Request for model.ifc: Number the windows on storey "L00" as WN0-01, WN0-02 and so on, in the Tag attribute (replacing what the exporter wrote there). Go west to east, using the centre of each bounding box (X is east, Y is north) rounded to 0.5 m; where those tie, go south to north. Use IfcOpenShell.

First a look at what the model holds.

```python
import ifcopenshell
import ifcopenshell.util.element
import ifcopenshell.util.placement

model = ifcopenshell.open("model.ifc")
print(model.schema)
storey = next(s for s in model.by_type("IfcBuildingStorey") if s.Name == "L00")
windows = [e for e in ifcopenshell.util.element.get_decomposition(storey) if e.is_a("IfcWindow")]
for e in sorted(windows, key=lambda e: e.id()):
    origin = ifcopenshell.util.placement.get_local_placement(e.ObjectPlacement)[:3, 3]
    print(e.id(), e.Tag, e.Name, origin.round(2) + 0.0, sep=" | ")
```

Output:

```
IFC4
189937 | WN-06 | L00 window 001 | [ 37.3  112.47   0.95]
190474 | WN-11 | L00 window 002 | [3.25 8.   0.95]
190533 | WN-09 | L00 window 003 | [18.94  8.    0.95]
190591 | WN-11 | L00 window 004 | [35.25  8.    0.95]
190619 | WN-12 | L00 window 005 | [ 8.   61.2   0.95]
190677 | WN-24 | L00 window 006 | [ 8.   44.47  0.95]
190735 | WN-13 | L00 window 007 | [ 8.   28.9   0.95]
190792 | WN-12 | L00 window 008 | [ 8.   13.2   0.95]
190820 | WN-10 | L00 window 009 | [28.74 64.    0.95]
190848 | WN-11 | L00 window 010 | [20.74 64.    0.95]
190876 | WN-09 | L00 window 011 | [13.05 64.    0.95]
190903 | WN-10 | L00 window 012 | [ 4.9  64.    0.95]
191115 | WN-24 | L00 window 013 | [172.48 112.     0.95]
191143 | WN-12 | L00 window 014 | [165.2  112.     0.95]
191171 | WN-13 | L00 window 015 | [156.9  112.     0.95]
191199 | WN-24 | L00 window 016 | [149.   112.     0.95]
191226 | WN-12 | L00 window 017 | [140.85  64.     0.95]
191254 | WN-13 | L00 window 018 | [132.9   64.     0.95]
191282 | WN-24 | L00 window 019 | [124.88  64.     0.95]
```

```python
import ifcopenshell
import ifcopenshell.geom
import ifcopenshell.util.element
import ifcopenshell.util.shape

model = ifcopenshell.open("model.ifc")
settings = ifcopenshell.geom.settings()
settings.set("use-world-coords", True)


def centre(element):
    shape = ifcopenshell.geom.create_shape(settings, element)
    return ifcopenshell.util.shape.get_bbox_centroid(shape.geometry)


storey = next(s for s in model.by_type("IfcBuildingStorey") if s.Name == "L00")
windows = [e for e in ifcopenshell.util.element.get_decomposition(storey) if e.is_a("IfcWindow")]

# Insertion points can sit at a corner or the storey origin, so sort by the geometry (in metres).
centres = {e: centre(e) for e in windows}
windows.sort(key=lambda e: (round(centres[e][0] / 0.5), centres[e][1]))

for i, e in enumerate(windows, start=1):
    number = f"WN0-{i:02d}"
    e.Tag = number
    print(e.id(), number)

model.write("model_edited.ifc")
```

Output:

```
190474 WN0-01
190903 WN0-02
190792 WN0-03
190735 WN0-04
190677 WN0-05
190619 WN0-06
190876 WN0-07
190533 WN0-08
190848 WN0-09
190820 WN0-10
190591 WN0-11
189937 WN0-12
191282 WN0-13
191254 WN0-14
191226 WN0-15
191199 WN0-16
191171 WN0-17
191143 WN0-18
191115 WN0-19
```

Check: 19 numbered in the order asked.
